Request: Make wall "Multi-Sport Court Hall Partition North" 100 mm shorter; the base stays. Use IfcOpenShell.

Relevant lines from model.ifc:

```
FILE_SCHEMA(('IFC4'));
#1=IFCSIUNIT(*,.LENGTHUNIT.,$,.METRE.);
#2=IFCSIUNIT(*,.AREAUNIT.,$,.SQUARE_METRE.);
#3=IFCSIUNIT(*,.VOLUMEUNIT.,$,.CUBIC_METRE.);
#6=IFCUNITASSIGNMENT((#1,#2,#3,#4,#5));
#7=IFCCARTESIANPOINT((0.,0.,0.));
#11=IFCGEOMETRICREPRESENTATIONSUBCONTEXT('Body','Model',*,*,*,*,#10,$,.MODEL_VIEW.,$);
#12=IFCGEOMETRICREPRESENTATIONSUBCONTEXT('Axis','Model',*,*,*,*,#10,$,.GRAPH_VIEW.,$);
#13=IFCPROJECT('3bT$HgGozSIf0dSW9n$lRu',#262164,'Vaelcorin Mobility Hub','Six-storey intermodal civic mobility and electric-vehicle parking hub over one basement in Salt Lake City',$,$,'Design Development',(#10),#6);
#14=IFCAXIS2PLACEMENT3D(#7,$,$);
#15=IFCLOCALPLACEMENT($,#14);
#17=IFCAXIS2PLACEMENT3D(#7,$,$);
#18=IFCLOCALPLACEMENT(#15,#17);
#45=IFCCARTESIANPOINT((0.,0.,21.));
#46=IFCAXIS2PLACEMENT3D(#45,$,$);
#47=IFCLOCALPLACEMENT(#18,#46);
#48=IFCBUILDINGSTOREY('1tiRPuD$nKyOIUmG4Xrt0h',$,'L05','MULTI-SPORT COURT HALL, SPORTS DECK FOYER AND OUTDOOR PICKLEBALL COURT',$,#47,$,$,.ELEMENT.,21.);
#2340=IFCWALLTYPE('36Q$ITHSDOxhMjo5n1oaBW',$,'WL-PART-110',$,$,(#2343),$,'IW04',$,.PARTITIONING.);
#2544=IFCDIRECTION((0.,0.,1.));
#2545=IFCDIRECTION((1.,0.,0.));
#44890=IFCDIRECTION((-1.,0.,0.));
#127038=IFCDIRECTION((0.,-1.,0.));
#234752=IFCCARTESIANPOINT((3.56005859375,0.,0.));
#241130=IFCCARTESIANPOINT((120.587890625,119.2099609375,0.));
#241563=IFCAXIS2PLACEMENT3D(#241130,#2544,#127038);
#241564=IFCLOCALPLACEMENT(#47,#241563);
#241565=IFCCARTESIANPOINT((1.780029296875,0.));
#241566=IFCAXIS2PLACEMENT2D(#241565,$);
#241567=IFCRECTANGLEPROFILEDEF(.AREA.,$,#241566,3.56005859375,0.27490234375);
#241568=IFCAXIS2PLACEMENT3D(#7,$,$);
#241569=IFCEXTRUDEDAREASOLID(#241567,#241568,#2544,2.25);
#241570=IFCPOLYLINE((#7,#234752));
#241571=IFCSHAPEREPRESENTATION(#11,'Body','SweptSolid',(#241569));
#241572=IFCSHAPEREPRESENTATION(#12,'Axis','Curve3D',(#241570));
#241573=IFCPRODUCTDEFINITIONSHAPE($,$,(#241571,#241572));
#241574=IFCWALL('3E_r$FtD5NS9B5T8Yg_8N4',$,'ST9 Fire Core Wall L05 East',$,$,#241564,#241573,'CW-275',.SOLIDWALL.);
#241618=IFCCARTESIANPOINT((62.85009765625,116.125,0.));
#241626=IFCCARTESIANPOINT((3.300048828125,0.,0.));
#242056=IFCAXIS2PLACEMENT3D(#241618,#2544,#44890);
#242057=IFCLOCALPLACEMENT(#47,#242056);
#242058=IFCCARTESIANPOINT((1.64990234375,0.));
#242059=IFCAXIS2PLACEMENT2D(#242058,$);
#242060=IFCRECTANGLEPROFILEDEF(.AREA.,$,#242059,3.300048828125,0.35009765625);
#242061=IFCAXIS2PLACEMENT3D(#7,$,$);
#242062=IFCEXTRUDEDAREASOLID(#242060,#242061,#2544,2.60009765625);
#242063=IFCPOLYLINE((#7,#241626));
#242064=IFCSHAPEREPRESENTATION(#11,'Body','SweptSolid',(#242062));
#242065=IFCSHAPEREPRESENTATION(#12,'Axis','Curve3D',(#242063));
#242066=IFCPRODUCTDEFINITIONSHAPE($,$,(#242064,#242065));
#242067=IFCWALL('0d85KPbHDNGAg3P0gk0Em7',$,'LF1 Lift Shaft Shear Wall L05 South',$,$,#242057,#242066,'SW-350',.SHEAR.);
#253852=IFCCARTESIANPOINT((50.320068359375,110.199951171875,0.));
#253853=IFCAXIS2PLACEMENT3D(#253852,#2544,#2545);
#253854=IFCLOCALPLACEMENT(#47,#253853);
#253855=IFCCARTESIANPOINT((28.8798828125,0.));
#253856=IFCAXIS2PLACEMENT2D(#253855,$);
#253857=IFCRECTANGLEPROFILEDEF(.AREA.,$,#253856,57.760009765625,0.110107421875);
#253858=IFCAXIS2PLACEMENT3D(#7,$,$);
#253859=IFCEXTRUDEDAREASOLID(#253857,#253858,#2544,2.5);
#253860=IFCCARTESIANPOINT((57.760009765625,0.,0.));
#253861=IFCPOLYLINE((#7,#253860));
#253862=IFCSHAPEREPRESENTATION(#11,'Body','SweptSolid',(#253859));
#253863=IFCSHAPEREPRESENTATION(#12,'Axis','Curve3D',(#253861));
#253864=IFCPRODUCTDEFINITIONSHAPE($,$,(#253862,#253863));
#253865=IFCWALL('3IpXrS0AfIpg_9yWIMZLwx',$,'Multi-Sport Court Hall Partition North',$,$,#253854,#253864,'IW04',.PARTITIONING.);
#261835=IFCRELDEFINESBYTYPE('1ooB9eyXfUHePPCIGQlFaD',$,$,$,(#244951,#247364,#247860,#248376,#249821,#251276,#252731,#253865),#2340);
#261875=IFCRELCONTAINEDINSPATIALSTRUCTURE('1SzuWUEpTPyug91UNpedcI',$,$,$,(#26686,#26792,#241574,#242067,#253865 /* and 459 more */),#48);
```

```python
import ifcopenshell
import ifcopenshell.geom
import ifcopenshell.util.representation
import ifcopenshell.util.shape
import ifcopenshell.util.unit

model = ifcopenshell.open("model.ifc")
unit_scale = ifcopenshell.util.unit.calculate_unit_scale(model)
settings = ifcopenshell.geom.settings()


def volume(element):
    """Net volume in cubic metres, openings subtracted."""
    shape = ifcopenshell.geom.create_shape(settings, element)
    return ifcopenshell.util.shape.get_volume(shape.geometry)


wall = model.by_guid("3IpXrS0AfIpg_9yWIMZLwx")
before = volume(wall)

body = ifcopenshell.util.representation.get_representation(wall, "Model", "Body")
solid = body.Items[0]
old_height = solid.Depth
solid.Depth -= 0.1 / unit_scale
after = volume(wall)

print(f"height {old_height:g} -> {solid.Depth:g}, volume {before:.3f} -> {after:.3f} m3")

model.write("model-out.ifc")
```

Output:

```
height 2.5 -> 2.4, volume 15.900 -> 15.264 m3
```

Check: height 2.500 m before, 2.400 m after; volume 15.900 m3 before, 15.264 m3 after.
